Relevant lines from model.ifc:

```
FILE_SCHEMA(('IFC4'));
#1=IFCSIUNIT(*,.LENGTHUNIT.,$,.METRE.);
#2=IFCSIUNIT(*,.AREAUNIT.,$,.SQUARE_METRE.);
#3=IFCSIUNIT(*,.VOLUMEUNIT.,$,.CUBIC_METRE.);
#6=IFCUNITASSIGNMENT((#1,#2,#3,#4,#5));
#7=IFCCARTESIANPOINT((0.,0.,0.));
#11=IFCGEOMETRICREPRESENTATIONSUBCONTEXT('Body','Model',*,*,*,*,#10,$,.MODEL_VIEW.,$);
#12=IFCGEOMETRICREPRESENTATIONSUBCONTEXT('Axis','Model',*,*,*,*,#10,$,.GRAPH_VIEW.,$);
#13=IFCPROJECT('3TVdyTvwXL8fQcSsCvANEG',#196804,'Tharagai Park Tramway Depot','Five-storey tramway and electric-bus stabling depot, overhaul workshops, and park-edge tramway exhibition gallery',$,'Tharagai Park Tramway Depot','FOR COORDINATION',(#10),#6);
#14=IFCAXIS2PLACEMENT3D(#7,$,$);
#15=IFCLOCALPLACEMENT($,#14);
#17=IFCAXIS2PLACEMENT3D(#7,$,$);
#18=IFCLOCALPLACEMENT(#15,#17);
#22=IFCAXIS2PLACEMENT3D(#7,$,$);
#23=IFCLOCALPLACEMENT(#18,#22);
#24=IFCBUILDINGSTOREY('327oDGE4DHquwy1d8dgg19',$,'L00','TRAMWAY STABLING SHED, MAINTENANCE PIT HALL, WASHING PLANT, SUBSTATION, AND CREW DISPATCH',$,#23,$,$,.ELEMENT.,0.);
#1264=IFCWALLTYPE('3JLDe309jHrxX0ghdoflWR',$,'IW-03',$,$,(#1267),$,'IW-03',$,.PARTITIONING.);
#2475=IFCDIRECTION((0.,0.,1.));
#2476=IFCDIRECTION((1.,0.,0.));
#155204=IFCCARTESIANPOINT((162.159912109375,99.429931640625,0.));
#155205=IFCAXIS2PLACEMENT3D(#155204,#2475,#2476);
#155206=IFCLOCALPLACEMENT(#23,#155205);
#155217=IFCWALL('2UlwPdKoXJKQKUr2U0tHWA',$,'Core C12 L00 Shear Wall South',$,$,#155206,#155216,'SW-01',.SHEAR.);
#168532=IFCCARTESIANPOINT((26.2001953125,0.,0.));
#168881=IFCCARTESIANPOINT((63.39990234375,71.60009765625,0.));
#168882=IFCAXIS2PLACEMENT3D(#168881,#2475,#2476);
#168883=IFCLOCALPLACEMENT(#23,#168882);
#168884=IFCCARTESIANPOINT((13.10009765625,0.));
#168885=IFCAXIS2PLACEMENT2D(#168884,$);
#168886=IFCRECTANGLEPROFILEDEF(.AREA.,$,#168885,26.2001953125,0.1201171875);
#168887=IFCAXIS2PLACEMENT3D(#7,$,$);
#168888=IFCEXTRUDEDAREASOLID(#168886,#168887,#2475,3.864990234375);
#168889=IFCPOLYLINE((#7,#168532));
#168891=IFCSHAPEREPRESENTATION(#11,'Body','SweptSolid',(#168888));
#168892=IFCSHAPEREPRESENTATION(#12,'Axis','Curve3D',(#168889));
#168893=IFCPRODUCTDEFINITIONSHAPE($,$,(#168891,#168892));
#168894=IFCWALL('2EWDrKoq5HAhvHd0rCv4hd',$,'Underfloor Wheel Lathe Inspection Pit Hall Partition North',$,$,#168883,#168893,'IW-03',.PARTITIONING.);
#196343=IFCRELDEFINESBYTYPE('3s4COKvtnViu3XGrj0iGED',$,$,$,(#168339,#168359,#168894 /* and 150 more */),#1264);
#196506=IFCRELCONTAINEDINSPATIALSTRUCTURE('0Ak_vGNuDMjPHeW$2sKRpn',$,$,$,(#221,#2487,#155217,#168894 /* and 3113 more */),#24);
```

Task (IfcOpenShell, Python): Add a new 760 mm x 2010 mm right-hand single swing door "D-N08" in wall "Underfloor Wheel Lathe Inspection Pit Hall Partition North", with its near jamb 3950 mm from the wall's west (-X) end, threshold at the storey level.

```python
import numpy as np
import ifcopenshell
import ifcopenshell.api.feature
import ifcopenshell.api.geometry
import ifcopenshell.api.root
import ifcopenshell.api.spatial
import ifcopenshell.geom
import ifcopenshell.util.element
import ifcopenshell.util.placement
import ifcopenshell.util.representation
import ifcopenshell.util.shape
import ifcopenshell.util.unit

model = ifcopenshell.open("model.ifc")
unit_scale = ifcopenshell.util.unit.calculate_unit_scale(model)
settings = ifcopenshell.geom.settings()


def volume(element):
    """Net volume in cubic metres, openings subtracted."""
    shape = ifcopenshell.geom.create_shape(settings, element)
    return ifcopenshell.util.shape.get_volume(shape.geometry)


wall = model.by_guid("2EWDrKoq5HAhvHd0rCv4hd")
storey = ifcopenshell.util.element.get_container(wall, ifc_class="IfcBuildingStorey")
context = ifcopenshell.util.representation.get_context(model, "Model", "Body", "MODEL_VIEW")
before = volume(wall)

width, height, from_end, sill = 0.76, 2.01, 3.95, 0.0  # metres

# The wall runs along its own X axis, and the end named is its -X end.
wall_shape = ifcopenshell.geom.create_shape(settings, wall)
x, y, z = ifcopenshell.util.shape.get_vertices(wall_shape.geometry).T
start = x.min() + from_end
face, thickness = float(y.min()), float(y.max() - y.min())
wall_matrix = ifcopenshell.util.placement.get_local_placement(wall.ObjectPlacement)
level = ifcopenshell.util.placement.get_local_placement(storey.ObjectPlacement)[2, 3]


def in_wall(x, y):
    """Placement at x, y metres in the wall's axes, at sill height."""
    matrix = wall_matrix.copy()
    matrix[:, 3] = wall_matrix @ np.array([x / unit_scale, y / unit_scale, 0.0, 1.0])
    matrix[2, 3] = level + sill / unit_scale
    return matrix


# Opening: a box that overshoots both wall faces by 50 mm.
opening = ifcopenshell.api.root.create_entity(model, ifc_class="IfcOpeningElement", predefined_type="OPENING")
box = ifcopenshell.api.geometry.add_wall_representation(
    model, context=context, length=width, height=height, thickness=thickness + 0.1
)
ifcopenshell.api.geometry.assign_representation(model, product=opening, representation=box)
ifcopenshell.api.geometry.edit_object_placement(model, product=opening, matrix=in_wall(start, face - 0.05), is_si=False)
ifcopenshell.api.feature.add_feature(model, feature=opening, element=wall)

door = ifcopenshell.api.root.create_entity(model, ifc_class="IfcDoor", name="D-N08", predefined_type="DOOR")
door.OverallWidth, door.OverallHeight = width / unit_scale, height / unit_scale
door.OperationType = "SINGLE_SWING_RIGHT"
body = ifcopenshell.api.geometry.add_door_representation(
    model,
    context=context,
    overall_width=door.OverallWidth,
    overall_height=door.OverallHeight,
    operation_type="SINGLE_SWING_RIGHT",
    lining_properties={"LiningDepth": thickness / unit_scale, "ThresholdDepth": thickness / unit_scale},
)
ifcopenshell.api.geometry.assign_representation(model, product=door, representation=body)
ifcopenshell.api.spatial.assign_container(model, products=[door], relating_structure=storey)
ifcopenshell.api.feature.add_filling(model, opening=opening, element=door)

# The lining spans the wall, so the door starts at the wall face.
ifcopenshell.api.geometry.edit_object_placement(model, product=door, matrix=in_wall(start, face), is_si=False)

after = volume(wall)

print(f"wall volume {before:.3f} -> {after:.3f} m3")

model.write("model_edited.ifc")
```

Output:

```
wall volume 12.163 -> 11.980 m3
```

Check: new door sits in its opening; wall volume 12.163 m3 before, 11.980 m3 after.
